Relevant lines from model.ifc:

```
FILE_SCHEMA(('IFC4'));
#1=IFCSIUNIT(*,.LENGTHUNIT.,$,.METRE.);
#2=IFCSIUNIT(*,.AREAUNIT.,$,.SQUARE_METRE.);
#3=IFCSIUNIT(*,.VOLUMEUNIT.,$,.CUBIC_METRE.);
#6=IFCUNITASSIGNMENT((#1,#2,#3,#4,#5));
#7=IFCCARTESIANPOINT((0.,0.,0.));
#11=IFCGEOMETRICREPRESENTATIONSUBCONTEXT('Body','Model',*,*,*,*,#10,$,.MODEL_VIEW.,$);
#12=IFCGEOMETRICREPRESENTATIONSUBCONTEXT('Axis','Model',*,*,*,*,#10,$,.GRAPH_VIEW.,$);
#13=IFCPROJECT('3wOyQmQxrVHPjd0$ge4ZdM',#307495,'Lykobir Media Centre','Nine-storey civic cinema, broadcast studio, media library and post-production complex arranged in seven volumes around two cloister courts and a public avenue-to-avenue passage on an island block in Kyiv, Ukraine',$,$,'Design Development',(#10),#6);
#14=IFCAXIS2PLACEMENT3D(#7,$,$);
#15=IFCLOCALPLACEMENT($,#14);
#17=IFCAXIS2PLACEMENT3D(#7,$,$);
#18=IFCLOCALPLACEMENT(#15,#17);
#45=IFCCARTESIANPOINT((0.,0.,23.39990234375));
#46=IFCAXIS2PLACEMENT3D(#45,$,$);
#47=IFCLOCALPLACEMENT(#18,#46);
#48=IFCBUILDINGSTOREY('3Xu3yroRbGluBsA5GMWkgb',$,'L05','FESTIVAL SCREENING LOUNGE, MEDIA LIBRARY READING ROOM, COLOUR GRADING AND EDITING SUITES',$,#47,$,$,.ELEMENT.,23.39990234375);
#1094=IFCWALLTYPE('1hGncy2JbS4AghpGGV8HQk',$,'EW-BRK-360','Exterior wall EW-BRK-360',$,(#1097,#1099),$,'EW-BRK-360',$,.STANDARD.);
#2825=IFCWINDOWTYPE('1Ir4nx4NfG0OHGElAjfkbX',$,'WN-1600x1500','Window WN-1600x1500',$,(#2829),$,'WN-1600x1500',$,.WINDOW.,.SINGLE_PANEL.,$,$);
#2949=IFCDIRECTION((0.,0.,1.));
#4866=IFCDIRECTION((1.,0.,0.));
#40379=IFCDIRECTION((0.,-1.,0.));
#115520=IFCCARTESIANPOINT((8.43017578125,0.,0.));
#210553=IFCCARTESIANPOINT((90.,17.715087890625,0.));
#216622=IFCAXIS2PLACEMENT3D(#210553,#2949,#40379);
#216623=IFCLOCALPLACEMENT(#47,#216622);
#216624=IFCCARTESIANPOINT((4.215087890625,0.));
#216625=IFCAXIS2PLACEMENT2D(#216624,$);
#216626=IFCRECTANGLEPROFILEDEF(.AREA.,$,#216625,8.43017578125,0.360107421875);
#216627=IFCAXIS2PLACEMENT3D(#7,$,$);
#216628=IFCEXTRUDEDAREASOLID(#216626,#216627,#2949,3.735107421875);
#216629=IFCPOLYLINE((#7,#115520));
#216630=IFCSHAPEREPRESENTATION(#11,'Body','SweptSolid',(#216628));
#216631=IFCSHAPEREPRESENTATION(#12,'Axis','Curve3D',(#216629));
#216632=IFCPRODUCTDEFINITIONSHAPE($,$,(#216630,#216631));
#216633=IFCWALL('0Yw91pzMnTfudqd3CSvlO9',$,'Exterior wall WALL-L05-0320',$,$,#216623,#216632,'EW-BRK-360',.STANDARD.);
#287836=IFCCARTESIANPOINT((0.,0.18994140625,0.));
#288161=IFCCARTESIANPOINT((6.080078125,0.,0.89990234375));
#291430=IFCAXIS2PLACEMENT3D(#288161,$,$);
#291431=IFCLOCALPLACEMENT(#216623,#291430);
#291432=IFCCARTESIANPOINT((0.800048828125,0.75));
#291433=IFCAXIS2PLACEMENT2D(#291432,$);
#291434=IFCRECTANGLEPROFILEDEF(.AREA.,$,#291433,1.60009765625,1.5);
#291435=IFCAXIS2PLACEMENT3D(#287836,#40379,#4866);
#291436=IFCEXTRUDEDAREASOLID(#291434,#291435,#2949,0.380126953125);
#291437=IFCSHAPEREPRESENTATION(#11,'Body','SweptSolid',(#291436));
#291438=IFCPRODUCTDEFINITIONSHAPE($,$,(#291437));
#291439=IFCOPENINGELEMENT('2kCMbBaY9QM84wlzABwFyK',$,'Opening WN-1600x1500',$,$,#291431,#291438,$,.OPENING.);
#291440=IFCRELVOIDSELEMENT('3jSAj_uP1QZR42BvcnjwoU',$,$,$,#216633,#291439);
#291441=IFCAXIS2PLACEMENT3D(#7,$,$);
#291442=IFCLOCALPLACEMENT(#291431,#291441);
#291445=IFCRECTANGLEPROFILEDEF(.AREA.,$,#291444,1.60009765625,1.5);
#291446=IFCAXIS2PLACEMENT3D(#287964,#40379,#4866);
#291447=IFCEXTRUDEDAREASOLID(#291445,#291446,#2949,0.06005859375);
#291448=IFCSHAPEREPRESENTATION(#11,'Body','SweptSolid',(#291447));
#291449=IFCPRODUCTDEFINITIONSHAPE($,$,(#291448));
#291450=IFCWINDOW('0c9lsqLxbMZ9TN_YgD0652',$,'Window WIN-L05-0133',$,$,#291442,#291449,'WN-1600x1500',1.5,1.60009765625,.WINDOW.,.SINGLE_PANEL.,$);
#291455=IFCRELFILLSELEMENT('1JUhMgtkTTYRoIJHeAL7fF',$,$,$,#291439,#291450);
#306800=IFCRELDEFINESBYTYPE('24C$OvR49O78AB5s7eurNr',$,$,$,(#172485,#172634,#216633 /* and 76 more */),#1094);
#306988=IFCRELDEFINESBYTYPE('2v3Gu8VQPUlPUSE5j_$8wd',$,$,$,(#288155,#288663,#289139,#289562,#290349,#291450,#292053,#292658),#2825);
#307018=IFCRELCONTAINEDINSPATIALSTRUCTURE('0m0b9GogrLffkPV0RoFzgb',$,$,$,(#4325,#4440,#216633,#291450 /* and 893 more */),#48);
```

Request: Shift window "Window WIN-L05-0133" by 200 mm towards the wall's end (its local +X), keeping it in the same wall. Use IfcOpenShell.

```python
import ifcopenshell
import ifcopenshell.api.geometry
import ifcopenshell.util.placement

model = ifcopenshell.open("model.ifc")

window = model.by_guid("0c9lsqLxbMZ9TN_YgD0652")
opening = window.FillsVoids[0].RelatingOpeningElement
wall = opening.VoidsElements[0].RelatingBuildingElement

wall_matrix = ifcopenshell.util.placement.get_local_placement(wall.ObjectPlacement)
shift = wall_matrix[:3, 0] * 0.2
before = ifcopenshell.util.placement.get_local_placement(window.ObjectPlacement)[:3, 3].copy()

# The window is placed relative to its opening, so it follows when the opening moves.
matrix = ifcopenshell.util.placement.get_local_placement(opening.ObjectPlacement)
matrix[:3, 3] += shift
ifcopenshell.api.geometry.edit_object_placement(
    model, product=opening, matrix=matrix, is_si=False, should_transform_children=True
)

after = ifcopenshell.util.placement.get_local_placement(window.ObjectPlacement)[:3, 3]
print("window moved by", (after - before).round(3) + 0.0)

model.write("model_updated.ifc")
```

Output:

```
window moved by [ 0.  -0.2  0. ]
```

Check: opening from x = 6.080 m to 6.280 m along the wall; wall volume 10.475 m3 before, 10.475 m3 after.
